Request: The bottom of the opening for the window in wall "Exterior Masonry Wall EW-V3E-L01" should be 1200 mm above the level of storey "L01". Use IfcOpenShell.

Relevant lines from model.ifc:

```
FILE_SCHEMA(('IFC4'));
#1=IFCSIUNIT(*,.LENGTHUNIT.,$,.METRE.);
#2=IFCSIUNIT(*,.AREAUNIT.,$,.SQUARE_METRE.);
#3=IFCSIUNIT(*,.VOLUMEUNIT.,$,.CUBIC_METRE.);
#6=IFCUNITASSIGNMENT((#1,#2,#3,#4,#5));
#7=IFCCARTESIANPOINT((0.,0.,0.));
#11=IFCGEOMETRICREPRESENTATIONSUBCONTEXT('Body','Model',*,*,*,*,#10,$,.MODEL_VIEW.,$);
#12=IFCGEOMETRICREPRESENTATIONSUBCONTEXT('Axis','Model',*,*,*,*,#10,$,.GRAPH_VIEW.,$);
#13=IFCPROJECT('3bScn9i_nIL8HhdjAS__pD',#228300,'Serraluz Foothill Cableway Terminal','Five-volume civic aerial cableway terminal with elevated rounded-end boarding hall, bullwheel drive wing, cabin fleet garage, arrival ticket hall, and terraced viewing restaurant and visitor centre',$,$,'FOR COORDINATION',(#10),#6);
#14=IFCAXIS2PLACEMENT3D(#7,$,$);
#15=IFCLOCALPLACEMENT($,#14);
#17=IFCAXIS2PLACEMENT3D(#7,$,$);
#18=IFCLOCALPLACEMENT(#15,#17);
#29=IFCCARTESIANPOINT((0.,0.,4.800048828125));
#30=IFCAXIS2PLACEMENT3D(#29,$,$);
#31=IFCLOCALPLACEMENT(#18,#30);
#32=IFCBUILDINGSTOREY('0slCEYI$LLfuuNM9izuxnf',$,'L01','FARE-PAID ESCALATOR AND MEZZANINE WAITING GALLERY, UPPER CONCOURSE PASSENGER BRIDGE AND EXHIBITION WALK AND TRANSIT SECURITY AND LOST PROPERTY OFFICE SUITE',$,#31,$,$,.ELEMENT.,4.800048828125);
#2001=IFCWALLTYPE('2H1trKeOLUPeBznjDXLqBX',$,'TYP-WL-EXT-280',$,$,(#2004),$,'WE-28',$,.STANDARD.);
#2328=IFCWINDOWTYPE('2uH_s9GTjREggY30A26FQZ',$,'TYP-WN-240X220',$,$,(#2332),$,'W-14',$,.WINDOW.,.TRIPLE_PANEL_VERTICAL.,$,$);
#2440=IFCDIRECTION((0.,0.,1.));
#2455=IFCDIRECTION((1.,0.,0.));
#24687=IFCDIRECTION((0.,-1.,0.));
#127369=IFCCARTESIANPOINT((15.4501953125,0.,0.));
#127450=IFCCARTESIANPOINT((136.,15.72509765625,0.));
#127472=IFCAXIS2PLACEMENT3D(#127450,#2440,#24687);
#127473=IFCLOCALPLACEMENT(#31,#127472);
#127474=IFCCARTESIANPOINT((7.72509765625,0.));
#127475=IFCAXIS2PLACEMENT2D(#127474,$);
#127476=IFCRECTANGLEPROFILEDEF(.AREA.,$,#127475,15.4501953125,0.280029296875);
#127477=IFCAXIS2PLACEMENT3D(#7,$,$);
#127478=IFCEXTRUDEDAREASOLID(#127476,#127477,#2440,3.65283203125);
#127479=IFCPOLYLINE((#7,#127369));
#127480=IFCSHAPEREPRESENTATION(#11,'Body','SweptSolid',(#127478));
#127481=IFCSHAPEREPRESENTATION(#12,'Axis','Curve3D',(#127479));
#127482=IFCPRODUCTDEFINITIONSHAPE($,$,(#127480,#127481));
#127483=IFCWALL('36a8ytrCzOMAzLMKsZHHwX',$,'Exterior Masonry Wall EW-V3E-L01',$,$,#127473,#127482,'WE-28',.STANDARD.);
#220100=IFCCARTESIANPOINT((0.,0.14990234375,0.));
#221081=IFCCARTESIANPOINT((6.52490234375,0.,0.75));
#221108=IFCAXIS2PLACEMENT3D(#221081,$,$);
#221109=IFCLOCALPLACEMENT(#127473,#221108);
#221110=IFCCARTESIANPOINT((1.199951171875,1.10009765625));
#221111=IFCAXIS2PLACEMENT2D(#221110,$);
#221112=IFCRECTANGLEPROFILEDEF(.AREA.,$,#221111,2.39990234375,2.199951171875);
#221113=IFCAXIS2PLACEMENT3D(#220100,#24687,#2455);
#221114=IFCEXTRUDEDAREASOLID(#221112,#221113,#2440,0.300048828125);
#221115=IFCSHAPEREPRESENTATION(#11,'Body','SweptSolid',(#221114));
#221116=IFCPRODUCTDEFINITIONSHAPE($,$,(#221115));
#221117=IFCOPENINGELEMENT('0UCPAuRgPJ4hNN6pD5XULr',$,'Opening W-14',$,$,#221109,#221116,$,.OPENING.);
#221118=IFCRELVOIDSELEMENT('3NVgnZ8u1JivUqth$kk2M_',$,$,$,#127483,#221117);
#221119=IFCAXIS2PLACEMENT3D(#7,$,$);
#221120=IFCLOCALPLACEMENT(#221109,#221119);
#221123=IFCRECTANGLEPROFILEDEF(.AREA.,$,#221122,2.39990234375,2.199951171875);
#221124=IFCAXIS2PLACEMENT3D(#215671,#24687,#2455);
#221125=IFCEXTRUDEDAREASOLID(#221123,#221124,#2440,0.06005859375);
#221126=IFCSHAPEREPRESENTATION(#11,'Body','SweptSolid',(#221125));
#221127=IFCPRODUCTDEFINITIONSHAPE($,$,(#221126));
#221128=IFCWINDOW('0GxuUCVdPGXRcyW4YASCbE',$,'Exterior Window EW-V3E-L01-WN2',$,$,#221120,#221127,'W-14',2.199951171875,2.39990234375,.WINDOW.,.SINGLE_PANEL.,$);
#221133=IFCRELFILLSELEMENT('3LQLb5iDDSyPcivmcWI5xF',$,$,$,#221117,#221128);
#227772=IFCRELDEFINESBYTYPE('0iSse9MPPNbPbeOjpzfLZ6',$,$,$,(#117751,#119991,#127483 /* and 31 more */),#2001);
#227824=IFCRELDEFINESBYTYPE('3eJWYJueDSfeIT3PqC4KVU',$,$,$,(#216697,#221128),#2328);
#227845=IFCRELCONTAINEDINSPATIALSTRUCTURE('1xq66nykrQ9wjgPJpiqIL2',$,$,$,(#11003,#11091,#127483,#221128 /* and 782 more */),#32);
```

```python
import numpy as np
import ifcopenshell
import ifcopenshell.api.geometry
import ifcopenshell.geom
import ifcopenshell.util.element
import ifcopenshell.util.placement
import ifcopenshell.util.shape
import ifcopenshell.util.unit

model = ifcopenshell.open("model.ifc")
unit_scale = ifcopenshell.util.unit.calculate_unit_scale(model)

window = model.by_guid("0GxuUCVdPGXRcyW4YASCbE")
opening = window.FillsVoids[0].RelatingOpeningElement
storey = ifcopenshell.util.element.get_container(window, ifc_class="IfcBuildingStorey")
level = ifcopenshell.util.placement.get_local_placement(storey.ObjectPlacement)[2, 3]

# The opening's origin need not be at the sill, so measure its lowest point.
shape = ifcopenshell.geom.create_shape(ifcopenshell.geom.settings(), opening)
bottom = ifcopenshell.util.shape.get_shape_bottom_elevation(shape, shape.geometry) / unit_scale
dz = level + 1.2 / unit_scale - bottom

shift = np.array([0.0, 0.0, dz])
# The window is placed relative to its opening, so it follows when the opening moves.
matrix = ifcopenshell.util.placement.get_local_placement(opening.ObjectPlacement)
matrix[:3, 3] += shift
ifcopenshell.api.geometry.edit_object_placement(
    model, product=opening, matrix=matrix, is_si=False, should_transform_children=True
)

print(f"moved by {dz * unit_scale:+.3f} m")

model.write("model_rev.ifc")
```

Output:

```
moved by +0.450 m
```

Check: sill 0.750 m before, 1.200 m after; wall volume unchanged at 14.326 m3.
